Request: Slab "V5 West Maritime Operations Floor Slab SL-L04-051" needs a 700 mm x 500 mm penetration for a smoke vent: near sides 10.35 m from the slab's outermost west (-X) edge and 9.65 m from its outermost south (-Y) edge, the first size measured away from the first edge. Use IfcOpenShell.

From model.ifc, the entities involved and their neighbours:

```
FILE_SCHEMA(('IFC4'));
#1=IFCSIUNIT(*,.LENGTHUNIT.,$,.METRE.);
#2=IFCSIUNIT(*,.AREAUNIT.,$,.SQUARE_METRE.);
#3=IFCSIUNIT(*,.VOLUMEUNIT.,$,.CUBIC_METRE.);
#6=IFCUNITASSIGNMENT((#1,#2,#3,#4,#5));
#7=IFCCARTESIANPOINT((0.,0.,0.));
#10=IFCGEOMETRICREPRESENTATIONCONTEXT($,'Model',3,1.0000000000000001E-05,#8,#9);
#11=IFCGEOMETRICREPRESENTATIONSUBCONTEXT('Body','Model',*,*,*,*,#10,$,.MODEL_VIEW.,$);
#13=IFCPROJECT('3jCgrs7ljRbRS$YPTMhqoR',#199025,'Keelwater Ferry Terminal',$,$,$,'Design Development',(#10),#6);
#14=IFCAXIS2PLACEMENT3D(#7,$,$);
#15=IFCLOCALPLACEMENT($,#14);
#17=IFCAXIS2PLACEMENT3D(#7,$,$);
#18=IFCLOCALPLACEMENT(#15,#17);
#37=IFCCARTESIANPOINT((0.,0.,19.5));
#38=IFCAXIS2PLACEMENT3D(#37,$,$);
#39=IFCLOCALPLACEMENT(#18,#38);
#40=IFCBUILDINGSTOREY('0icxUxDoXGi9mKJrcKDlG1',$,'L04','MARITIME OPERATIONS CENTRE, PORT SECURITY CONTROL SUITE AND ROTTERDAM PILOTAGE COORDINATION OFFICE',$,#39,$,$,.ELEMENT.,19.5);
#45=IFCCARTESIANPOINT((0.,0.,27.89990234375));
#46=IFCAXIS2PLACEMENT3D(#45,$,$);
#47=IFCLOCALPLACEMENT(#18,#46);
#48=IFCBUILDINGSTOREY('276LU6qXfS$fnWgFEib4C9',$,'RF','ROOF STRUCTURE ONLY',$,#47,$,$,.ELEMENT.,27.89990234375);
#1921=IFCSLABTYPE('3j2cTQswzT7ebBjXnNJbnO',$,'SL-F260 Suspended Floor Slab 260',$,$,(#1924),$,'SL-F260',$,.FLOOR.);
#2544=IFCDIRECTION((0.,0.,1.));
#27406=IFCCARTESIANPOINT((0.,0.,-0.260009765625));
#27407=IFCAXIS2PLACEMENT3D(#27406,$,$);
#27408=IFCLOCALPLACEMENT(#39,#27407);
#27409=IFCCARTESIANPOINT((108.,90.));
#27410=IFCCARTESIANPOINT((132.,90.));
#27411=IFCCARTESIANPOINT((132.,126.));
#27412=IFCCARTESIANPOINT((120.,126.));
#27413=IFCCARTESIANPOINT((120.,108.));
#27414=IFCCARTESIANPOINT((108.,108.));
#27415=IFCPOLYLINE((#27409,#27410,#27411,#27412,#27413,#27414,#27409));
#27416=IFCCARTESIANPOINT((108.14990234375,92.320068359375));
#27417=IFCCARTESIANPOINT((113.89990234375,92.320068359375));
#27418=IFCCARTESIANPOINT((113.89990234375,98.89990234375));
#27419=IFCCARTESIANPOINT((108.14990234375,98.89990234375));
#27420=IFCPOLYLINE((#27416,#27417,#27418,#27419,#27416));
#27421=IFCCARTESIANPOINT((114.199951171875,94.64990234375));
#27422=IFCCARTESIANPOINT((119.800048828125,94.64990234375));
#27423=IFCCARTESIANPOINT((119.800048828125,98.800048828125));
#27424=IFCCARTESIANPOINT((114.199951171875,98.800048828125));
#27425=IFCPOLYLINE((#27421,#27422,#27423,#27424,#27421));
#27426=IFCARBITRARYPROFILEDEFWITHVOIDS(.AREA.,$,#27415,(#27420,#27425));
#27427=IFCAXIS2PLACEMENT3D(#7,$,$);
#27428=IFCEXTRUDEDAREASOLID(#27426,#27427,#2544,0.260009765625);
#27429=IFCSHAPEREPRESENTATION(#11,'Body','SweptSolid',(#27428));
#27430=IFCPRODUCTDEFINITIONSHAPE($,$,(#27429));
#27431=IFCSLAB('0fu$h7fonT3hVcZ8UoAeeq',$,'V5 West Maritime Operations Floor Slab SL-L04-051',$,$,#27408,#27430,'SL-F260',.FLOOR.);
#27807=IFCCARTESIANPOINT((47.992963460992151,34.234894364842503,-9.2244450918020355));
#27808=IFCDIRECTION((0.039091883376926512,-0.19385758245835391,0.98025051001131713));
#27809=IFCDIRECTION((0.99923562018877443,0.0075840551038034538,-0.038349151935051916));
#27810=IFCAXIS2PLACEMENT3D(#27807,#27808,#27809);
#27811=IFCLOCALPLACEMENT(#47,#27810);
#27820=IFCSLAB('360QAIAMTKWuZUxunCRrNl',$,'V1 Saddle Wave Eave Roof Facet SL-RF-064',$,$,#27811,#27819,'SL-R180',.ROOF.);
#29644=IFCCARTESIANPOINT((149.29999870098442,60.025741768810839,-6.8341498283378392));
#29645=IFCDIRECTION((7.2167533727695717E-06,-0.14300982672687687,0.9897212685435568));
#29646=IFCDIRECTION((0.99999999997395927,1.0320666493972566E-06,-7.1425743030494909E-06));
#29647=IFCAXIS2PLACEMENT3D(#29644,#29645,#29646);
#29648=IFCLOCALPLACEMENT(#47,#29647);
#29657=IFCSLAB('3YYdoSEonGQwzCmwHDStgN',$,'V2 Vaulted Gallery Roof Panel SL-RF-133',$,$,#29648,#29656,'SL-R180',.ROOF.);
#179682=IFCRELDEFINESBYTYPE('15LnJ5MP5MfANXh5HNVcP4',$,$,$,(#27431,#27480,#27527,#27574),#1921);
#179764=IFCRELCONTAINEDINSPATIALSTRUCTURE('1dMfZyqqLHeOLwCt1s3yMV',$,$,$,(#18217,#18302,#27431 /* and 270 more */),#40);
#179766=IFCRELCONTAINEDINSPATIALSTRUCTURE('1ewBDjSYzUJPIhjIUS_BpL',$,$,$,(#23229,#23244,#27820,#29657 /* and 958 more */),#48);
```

```python
import numpy as np
import ifcopenshell
import ifcopenshell.api.feature
import ifcopenshell.api.geometry
import ifcopenshell.api.root
import ifcopenshell.geom
import ifcopenshell.util.placement
import ifcopenshell.util.representation
import ifcopenshell.util.shape
import ifcopenshell.util.unit

model = ifcopenshell.open("model.ifc")
unit_scale = ifcopenshell.util.unit.calculate_unit_scale(model)
settings = ifcopenshell.geom.settings()


def volume(element):
    """Net volume in cubic metres, openings subtracted."""
    shape = ifcopenshell.geom.create_shape(settings, element)
    return ifcopenshell.util.shape.get_volume(shape.geometry)


slab = model.by_id(27431)
before = volume(slab)

# Extent in the slab's own axes, in metres. The edges named are its -X and -Y sides.
slab_shape = ifcopenshell.geom.create_shape(settings, slab)
vertices = ifcopenshell.util.shape.get_vertices(slab_shape.geometry)
x_min, y_min, bottom = vertices.min(axis=0)
top = vertices[:, 2].max()

opening = ifcopenshell.api.root.create_entity(model, ifc_class="IfcOpeningElement", name="Smoke vent opening", predefined_type="OPENING")
context = ifcopenshell.util.representation.get_context(model, "Model", "Body", "MODEL_VIEW")
width, depth = 0.7, 0.5
outline = [(0.0, 0.0), (width, 0.0), (width, depth), (0.0, depth), (0.0, 0.0)]
# Overshoot both faces by 50 mm so the cut is clean.
shape = ifcopenshell.api.geometry.add_slab_representation(
    model, context=context, depth=top - bottom + 0.1, polyline=outline
)
ifcopenshell.api.geometry.assign_representation(model, product=opening, representation=shape)

matrix = ifcopenshell.util.placement.get_local_placement(slab.ObjectPlacement)
matrix[:, 3] = matrix @ np.append(np.array([x_min + 10.35, y_min + 9.65, bottom - 0.05]) / unit_scale, 1.0)
ifcopenshell.api.geometry.edit_object_placement(model, product=opening, matrix=matrix, is_si=False)
ifcopenshell.api.feature.add_feature(model, feature=opening, element=slab)

after = volume(slab)

print(f"slab volume {before:.3f} -> {after:.3f} m3")

model.write("model-out.ifc")
```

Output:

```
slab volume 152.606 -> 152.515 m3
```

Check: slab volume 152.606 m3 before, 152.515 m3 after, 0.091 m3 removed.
